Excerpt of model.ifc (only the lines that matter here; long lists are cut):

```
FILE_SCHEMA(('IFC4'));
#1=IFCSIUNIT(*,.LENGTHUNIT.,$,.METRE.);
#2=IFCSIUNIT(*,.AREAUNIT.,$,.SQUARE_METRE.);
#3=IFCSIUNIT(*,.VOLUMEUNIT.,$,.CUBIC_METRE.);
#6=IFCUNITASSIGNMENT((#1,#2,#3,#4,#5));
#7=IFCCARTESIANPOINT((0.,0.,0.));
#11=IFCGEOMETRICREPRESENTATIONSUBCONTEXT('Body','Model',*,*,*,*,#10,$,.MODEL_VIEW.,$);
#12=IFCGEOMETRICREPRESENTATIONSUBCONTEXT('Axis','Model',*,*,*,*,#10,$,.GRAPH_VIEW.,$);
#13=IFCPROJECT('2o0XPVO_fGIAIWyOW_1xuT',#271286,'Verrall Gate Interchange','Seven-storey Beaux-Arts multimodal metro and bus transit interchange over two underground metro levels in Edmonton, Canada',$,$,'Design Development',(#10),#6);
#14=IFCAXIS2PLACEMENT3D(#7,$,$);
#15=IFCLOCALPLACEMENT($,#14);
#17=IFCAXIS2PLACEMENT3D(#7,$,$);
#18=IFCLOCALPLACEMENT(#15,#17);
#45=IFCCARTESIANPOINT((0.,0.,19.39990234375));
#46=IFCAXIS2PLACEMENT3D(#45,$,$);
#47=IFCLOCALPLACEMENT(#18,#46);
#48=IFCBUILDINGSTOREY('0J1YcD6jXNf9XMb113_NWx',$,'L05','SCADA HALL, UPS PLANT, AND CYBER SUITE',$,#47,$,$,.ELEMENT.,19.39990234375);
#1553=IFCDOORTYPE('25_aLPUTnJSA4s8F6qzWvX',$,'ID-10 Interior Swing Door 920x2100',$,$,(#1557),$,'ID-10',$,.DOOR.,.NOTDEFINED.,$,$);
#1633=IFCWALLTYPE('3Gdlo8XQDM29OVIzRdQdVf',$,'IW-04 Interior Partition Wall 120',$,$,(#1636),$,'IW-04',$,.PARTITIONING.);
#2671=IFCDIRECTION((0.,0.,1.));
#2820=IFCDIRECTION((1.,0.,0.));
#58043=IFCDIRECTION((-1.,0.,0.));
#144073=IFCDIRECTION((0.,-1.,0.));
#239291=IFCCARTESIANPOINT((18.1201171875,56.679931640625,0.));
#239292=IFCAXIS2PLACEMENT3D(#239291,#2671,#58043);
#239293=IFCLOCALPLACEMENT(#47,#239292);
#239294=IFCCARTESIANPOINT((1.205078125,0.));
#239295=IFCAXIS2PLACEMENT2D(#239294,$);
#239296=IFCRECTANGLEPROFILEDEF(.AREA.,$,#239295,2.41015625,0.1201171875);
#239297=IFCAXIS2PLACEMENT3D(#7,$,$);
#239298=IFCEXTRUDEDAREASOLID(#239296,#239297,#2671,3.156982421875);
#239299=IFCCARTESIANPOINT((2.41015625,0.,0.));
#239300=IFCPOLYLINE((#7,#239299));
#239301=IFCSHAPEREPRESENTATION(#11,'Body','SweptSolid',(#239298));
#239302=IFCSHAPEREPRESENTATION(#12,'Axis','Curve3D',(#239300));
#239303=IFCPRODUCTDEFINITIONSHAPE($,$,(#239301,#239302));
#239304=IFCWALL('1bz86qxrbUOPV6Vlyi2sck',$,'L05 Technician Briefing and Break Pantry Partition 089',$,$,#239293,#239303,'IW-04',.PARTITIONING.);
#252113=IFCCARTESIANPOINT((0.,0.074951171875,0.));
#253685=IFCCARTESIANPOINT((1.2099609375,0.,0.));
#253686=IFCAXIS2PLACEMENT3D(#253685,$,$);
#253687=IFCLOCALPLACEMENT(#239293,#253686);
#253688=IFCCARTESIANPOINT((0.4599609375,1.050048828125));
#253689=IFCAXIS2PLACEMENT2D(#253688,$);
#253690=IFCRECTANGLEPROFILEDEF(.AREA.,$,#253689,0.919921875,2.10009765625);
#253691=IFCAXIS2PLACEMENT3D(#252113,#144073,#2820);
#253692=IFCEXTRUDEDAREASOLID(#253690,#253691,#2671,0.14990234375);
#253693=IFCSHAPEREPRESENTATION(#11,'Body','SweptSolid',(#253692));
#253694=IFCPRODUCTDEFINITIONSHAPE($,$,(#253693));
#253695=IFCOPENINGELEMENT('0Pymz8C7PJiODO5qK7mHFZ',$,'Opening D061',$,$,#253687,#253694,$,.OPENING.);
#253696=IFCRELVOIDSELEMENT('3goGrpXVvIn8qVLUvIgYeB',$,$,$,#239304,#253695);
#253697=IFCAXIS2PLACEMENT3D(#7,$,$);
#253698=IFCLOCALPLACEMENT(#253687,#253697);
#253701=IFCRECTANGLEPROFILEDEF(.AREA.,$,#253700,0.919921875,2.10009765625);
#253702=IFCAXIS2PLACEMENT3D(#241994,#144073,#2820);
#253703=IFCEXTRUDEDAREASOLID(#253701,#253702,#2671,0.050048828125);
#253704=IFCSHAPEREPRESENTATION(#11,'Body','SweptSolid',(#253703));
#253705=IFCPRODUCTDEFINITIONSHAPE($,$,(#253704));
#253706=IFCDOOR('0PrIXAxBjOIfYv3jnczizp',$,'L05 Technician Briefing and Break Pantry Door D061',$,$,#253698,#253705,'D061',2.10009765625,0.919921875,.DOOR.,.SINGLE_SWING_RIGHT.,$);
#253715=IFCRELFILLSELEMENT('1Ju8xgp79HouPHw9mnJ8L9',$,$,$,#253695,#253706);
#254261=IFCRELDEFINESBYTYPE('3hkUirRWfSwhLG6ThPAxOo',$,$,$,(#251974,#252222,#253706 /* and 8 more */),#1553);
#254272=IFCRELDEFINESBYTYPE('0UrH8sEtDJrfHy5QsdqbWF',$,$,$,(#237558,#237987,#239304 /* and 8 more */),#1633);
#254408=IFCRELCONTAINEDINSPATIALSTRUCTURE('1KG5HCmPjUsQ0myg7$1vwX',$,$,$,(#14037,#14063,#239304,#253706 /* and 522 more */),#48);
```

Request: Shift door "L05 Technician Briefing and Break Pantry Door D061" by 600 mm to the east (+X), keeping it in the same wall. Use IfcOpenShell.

```python
import ifcopenshell
import ifcopenshell.api.geometry
import ifcopenshell.util.placement
import ifcopenshell.util.unit

model = ifcopenshell.open("model.ifc")
unit_scale = ifcopenshell.util.unit.calculate_unit_scale(model)

door = model.by_id(253706)
opening = door.FillsVoids[0].RelatingOpeningElement
wall = opening.VoidsElements[0].RelatingBuildingElement

wall_matrix = ifcopenshell.util.placement.get_local_placement(wall.ObjectPlacement)
shift = wall_matrix[:3, 0] * -0.6 / unit_scale
before = ifcopenshell.util.placement.get_local_placement(door.ObjectPlacement)[:3, 3].copy()

# The door is placed relative to its opening, so it follows when the opening moves.
matrix = ifcopenshell.util.placement.get_local_placement(opening.ObjectPlacement)
matrix[:3, 3] += shift
ifcopenshell.api.geometry.edit_object_placement(
    model, product=opening, matrix=matrix, is_si=False, should_transform_children=True
)

after = ifcopenshell.util.placement.get_local_placement(door.ObjectPlacement)[:3, 3]
print("door moved by", (after - before).round(3) + 0.0)

model.write("model_edited.ifc")
```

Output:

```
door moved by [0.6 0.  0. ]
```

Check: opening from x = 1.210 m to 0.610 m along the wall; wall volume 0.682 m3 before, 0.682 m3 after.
